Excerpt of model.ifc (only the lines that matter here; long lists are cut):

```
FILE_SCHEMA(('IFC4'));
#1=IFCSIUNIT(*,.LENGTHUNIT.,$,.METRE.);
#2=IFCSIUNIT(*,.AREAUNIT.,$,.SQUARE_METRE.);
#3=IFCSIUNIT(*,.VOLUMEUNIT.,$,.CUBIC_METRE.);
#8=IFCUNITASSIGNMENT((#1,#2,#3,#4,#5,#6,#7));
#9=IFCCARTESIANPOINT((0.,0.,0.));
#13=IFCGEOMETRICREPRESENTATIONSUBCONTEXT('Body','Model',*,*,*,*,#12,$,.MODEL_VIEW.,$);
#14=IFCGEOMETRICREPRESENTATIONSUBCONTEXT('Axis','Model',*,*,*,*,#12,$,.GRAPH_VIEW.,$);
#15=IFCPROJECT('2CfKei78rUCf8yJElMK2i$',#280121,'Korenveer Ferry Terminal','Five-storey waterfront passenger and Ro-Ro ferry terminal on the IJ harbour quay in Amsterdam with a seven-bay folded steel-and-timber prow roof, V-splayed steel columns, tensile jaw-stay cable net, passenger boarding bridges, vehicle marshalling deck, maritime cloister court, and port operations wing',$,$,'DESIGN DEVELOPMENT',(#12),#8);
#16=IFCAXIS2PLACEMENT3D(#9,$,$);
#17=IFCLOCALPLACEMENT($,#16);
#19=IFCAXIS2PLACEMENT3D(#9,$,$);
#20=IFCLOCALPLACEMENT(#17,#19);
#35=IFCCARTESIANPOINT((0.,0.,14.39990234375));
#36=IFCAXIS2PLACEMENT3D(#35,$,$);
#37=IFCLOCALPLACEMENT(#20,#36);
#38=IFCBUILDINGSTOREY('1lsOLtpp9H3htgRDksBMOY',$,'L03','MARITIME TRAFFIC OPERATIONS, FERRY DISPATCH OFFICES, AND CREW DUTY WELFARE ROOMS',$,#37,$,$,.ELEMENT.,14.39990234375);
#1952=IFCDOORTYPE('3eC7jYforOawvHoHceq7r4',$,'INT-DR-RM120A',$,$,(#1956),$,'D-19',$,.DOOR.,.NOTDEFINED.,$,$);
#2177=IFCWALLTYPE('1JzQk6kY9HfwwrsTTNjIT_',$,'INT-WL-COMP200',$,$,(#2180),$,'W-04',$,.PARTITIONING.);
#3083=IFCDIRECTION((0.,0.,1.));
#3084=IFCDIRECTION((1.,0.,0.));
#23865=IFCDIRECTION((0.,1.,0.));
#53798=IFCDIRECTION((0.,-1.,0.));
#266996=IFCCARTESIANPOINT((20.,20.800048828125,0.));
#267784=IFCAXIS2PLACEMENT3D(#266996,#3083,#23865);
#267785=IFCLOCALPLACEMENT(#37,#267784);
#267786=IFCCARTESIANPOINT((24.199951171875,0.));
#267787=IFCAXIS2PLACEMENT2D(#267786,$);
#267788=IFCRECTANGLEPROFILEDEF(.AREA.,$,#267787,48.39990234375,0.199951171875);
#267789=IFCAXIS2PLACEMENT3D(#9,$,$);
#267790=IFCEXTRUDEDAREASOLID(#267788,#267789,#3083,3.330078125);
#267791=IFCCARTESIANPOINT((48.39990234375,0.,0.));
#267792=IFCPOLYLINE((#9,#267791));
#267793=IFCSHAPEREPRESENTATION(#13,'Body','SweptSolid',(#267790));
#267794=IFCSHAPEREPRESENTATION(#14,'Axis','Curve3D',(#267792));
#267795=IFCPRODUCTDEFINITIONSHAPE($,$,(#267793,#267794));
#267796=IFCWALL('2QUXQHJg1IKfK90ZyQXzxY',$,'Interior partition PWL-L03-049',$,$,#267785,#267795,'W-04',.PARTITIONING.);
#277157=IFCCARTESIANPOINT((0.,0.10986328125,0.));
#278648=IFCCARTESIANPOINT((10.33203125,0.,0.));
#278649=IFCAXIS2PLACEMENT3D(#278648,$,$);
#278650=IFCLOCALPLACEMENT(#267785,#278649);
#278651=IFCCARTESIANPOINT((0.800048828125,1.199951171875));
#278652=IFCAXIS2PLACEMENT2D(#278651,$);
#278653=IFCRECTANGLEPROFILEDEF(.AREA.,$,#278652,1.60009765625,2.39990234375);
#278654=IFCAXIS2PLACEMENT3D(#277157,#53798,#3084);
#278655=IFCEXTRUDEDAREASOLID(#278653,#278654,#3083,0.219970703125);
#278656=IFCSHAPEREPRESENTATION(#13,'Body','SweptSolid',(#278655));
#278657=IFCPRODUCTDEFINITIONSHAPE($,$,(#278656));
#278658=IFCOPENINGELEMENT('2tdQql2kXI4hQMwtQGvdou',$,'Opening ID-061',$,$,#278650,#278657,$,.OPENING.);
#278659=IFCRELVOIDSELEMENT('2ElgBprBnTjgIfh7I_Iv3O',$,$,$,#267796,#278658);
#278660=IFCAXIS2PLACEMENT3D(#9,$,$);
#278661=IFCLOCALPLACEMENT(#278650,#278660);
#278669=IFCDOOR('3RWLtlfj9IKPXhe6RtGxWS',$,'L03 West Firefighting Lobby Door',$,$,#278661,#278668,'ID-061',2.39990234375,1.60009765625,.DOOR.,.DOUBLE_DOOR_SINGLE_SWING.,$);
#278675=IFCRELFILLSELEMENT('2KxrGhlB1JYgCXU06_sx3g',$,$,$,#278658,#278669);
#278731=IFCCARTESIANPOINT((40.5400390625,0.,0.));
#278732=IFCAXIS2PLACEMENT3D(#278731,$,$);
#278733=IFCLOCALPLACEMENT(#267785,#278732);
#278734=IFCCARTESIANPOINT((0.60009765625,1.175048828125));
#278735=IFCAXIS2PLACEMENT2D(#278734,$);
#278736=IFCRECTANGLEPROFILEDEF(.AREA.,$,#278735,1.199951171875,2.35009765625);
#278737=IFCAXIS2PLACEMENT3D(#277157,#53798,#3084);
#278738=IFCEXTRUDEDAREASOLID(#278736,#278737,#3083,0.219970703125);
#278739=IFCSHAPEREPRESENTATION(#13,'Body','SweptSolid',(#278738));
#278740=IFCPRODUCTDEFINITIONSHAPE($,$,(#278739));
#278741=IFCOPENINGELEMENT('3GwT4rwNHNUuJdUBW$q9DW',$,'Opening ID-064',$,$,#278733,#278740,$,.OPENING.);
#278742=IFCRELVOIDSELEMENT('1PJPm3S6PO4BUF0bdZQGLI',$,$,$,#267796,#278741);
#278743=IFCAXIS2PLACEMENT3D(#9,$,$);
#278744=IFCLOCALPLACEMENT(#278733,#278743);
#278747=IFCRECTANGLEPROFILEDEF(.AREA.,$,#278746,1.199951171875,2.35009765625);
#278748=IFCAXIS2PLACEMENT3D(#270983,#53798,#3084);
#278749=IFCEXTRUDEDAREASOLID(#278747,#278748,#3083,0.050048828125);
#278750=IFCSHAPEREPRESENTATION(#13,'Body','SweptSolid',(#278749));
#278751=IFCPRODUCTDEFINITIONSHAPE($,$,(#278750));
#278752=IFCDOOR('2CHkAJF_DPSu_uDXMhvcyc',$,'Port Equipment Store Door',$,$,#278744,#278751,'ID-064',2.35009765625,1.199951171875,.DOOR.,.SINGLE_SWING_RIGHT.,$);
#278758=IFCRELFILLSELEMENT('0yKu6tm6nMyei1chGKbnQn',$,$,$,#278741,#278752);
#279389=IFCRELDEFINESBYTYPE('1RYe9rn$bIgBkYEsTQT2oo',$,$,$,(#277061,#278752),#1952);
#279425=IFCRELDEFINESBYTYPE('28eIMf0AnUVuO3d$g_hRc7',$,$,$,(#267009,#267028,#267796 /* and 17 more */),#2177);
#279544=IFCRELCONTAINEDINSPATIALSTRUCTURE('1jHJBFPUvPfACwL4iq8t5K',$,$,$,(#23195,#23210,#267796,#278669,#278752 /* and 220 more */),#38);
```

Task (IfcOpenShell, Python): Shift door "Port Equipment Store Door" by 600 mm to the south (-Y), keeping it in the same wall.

```python
import ifcopenshell
import ifcopenshell.api.geometry
import ifcopenshell.util.placement
import ifcopenshell.util.unit

model = ifcopenshell.open("model.ifc")
unit_scale = ifcopenshell.util.unit.calculate_unit_scale(model)

door = model.by_guid("2CHkAJF_DPSu_uDXMhvcyc")
opening = door.FillsVoids[0].RelatingOpeningElement
wall = opening.VoidsElements[0].RelatingBuildingElement

wall_matrix = ifcopenshell.util.placement.get_local_placement(wall.ObjectPlacement)
shift = wall_matrix[:3, 0] * -0.6 / unit_scale
before = ifcopenshell.util.placement.get_local_placement(door.ObjectPlacement)[:3, 3].copy()

# The door is placed relative to its opening, so it follows when the opening moves.
matrix = ifcopenshell.util.placement.get_local_placement(opening.ObjectPlacement)
matrix[:3, 3] += shift
ifcopenshell.api.geometry.edit_object_placement(
    model, product=opening, matrix=matrix, is_si=False, should_transform_children=True
)

after = ifcopenshell.util.placement.get_local_placement(door.ObjectPlacement)[:3, 3]
print("door moved by", (after - before).round(3) + 0.0)

model.write("model_edited.ifc")
```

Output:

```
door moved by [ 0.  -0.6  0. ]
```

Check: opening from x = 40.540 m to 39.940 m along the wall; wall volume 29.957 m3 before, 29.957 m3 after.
